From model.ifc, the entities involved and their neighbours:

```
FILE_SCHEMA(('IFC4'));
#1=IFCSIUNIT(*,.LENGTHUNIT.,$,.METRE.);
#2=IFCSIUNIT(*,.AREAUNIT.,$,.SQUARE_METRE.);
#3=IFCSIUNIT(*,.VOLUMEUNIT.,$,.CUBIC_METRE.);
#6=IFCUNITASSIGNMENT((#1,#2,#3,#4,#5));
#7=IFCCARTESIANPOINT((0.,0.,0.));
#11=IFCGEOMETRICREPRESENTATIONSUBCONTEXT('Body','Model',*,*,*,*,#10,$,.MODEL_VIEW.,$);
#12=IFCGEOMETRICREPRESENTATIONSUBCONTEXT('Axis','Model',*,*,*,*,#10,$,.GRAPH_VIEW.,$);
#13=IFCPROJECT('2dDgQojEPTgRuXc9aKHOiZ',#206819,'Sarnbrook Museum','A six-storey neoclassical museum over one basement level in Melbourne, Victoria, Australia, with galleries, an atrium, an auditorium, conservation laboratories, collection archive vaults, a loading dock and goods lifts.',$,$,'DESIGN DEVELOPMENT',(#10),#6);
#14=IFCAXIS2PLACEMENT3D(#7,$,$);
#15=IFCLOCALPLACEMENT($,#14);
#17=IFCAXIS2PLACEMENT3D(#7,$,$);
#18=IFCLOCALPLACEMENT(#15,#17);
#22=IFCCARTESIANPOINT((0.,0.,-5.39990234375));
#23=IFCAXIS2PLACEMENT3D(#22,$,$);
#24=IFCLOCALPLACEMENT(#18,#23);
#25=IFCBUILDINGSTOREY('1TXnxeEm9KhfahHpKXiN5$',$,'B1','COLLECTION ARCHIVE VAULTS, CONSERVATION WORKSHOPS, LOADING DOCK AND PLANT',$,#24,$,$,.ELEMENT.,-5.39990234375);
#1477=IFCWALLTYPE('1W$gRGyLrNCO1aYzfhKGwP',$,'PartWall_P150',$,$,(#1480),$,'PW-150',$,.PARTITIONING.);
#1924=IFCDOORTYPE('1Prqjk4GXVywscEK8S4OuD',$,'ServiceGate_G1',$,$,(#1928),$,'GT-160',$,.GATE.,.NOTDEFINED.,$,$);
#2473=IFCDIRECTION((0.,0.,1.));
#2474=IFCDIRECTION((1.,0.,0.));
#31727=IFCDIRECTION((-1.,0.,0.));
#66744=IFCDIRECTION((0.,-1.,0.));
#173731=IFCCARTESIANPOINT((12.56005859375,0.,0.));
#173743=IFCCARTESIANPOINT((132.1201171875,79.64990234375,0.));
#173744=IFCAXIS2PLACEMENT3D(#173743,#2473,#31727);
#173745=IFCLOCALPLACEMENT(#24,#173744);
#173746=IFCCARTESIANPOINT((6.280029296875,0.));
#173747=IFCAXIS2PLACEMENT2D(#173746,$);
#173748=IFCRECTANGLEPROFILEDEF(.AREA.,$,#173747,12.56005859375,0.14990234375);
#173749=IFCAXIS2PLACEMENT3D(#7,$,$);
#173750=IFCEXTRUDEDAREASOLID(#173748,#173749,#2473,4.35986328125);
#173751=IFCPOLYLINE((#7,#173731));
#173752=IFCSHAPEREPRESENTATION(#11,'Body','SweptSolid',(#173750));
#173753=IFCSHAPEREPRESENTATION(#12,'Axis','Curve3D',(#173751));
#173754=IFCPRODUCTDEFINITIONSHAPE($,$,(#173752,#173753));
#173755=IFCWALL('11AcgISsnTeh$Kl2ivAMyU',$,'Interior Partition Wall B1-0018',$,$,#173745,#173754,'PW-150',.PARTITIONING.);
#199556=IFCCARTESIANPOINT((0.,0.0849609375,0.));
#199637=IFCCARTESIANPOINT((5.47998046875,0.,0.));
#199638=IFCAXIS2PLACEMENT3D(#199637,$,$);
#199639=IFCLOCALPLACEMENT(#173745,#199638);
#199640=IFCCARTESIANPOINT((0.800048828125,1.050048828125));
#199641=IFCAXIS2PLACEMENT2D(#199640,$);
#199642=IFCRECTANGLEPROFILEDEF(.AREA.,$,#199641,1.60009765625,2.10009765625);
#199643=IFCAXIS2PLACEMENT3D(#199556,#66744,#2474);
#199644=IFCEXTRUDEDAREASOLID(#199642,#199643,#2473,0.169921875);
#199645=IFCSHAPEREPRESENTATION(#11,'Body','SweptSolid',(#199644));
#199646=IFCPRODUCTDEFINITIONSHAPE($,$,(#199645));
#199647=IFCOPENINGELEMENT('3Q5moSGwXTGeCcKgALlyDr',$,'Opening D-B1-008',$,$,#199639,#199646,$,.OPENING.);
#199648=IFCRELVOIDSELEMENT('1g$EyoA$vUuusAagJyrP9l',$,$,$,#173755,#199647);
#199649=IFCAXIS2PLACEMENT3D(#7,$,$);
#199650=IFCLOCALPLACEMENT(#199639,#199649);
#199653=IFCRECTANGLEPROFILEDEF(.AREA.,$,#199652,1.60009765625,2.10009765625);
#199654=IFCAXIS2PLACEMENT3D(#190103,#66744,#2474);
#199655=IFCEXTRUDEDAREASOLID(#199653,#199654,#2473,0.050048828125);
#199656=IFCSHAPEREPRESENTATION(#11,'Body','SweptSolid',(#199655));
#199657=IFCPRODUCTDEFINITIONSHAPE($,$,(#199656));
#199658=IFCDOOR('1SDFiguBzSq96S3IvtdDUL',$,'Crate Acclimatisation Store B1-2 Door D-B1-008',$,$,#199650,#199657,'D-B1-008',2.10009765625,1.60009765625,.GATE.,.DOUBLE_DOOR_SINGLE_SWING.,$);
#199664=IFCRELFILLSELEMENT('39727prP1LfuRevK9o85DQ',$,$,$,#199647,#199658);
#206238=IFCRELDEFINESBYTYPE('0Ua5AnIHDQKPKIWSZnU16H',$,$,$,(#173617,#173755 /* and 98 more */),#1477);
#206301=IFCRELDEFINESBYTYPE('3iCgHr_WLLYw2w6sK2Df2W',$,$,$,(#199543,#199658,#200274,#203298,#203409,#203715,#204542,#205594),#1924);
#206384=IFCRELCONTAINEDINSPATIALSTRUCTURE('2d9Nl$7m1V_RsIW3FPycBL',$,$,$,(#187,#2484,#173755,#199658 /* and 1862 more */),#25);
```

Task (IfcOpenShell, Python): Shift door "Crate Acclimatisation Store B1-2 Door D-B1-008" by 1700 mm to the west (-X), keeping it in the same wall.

```python
import ifcopenshell
import ifcopenshell.api.geometry
import ifcopenshell.util.placement
import ifcopenshell.util.unit

model = ifcopenshell.open("model.ifc")
unit_scale = ifcopenshell.util.unit.calculate_unit_scale(model)

door = model.by_guid("1SDFiguBzSq96S3IvtdDUL")
opening = door.FillsVoids[0].RelatingOpeningElement
wall = opening.VoidsElements[0].RelatingBuildingElement

wall_matrix = ifcopenshell.util.placement.get_local_placement(wall.ObjectPlacement)
shift = wall_matrix[:3, 0] * 1.7 / unit_scale
before = ifcopenshell.util.placement.get_local_placement(door.ObjectPlacement)[:3, 3].copy()

# The door is placed relative to its opening, so it follows when the opening moves.
matrix = ifcopenshell.util.placement.get_local_placement(opening.ObjectPlacement)
matrix[:3, 3] += shift
ifcopenshell.api.geometry.edit_object_placement(
    model, product=opening, matrix=matrix, is_si=False, should_transform_children=True
)

after = ifcopenshell.util.placement.get_local_placement(door.ObjectPlacement)[:3, 3]
print("door moved by", (after - before).round(3) + 0.0)

model.write("model-out.ifc")
```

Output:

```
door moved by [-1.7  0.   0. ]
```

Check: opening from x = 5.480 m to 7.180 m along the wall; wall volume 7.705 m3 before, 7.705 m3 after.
